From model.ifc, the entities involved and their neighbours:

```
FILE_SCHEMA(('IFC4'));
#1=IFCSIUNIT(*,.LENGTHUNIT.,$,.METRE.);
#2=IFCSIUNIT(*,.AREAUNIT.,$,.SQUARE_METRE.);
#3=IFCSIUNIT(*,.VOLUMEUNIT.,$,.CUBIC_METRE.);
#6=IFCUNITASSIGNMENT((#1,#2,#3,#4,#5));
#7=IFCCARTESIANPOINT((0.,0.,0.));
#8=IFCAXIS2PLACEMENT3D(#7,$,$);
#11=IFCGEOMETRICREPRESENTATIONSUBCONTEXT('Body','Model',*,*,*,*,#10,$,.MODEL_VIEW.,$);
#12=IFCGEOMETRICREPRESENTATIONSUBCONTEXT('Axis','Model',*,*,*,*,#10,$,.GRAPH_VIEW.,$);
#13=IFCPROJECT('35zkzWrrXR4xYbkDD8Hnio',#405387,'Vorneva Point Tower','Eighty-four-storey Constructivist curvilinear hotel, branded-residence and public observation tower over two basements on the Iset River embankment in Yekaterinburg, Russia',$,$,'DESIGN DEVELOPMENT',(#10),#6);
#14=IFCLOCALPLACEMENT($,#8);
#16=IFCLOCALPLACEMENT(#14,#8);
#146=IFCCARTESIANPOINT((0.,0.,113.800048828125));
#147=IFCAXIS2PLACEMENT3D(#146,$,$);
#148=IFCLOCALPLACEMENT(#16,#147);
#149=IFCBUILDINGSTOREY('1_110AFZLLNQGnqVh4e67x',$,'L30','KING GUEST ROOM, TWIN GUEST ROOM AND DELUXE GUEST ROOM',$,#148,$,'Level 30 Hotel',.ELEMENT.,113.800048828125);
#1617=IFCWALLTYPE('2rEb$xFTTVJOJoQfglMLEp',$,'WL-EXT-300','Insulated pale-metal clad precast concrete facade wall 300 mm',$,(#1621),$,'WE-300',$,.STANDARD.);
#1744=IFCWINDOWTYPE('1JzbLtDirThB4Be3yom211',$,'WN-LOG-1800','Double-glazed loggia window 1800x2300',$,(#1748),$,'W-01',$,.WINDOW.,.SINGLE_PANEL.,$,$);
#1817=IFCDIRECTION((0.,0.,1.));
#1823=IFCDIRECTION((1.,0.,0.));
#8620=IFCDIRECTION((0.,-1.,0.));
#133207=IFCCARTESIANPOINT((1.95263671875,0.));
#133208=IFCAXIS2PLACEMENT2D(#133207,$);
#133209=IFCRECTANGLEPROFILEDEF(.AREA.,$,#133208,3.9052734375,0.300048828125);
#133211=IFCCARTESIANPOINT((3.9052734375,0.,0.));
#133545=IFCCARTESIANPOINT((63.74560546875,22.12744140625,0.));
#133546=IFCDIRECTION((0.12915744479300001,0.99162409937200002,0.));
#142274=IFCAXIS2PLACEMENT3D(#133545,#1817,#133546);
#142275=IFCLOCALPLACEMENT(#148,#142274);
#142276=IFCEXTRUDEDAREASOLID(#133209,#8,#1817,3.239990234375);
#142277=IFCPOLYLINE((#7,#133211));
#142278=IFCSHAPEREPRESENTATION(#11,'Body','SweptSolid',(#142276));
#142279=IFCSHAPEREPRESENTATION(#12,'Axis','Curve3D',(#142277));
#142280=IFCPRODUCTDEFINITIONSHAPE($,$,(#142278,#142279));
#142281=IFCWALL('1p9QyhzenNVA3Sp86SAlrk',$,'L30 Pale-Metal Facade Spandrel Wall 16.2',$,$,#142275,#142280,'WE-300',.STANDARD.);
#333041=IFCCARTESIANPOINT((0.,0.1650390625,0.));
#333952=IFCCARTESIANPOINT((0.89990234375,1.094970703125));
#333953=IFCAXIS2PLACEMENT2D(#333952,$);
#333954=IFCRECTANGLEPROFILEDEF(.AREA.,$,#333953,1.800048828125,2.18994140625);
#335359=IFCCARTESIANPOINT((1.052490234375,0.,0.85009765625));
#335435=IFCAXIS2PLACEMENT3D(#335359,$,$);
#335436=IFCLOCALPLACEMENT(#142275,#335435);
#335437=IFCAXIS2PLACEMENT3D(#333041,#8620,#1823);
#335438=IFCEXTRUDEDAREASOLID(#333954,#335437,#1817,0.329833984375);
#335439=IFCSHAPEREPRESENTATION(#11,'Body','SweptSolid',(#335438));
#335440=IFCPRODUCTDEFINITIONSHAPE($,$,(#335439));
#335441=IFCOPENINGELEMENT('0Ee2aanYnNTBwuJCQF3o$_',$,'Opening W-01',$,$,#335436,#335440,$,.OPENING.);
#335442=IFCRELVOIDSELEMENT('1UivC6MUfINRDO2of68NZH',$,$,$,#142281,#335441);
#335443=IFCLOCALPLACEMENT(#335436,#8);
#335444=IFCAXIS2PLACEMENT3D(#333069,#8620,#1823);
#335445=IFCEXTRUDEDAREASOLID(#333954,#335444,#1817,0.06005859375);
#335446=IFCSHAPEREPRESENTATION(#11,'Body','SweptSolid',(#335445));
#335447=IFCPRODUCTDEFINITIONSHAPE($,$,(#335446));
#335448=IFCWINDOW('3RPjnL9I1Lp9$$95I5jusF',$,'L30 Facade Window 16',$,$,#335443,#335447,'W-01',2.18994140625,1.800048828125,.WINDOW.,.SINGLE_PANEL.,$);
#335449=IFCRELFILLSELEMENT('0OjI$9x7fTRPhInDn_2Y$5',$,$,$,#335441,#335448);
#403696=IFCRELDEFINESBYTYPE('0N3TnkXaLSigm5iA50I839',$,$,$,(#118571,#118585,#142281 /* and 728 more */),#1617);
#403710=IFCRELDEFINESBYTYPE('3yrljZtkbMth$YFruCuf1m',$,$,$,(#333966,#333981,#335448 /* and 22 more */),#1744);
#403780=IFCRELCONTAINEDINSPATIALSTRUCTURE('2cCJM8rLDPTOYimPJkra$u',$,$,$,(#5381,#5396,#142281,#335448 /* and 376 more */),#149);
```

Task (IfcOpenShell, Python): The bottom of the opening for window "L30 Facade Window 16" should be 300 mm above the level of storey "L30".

```python
import numpy as np
import ifcopenshell
import ifcopenshell.api.geometry
import ifcopenshell.geom
import ifcopenshell.util.element
import ifcopenshell.util.placement
import ifcopenshell.util.shape
import ifcopenshell.util.unit

model = ifcopenshell.open("model.ifc")
unit_scale = ifcopenshell.util.unit.calculate_unit_scale(model)

window = model.by_guid("3RPjnL9I1Lp9$$95I5jusF")
opening = window.FillsVoids[0].RelatingOpeningElement
storey = ifcopenshell.util.element.get_container(window, ifc_class="IfcBuildingStorey")
level = ifcopenshell.util.placement.get_local_placement(storey.ObjectPlacement)[2, 3]

# The opening's origin need not be at the sill, so measure its lowest point.
shape = ifcopenshell.geom.create_shape(ifcopenshell.geom.settings(), opening)
bottom = ifcopenshell.util.shape.get_shape_bottom_elevation(shape, shape.geometry) / unit_scale
dz = level + 0.3 / unit_scale - bottom

shift = np.array([0.0, 0.0, dz])
# The window is placed relative to its opening, so it follows when the opening moves.
matrix = ifcopenshell.util.placement.get_local_placement(opening.ObjectPlacement)
matrix[:3, 3] += shift
ifcopenshell.api.geometry.edit_object_placement(
    model, product=opening, matrix=matrix, is_si=False, should_transform_children=True
)

print(f"moved by {dz * unit_scale:+.3f} m")

model.write("model_rev.ifc")
```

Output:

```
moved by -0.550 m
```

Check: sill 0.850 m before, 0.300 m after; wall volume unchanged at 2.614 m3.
